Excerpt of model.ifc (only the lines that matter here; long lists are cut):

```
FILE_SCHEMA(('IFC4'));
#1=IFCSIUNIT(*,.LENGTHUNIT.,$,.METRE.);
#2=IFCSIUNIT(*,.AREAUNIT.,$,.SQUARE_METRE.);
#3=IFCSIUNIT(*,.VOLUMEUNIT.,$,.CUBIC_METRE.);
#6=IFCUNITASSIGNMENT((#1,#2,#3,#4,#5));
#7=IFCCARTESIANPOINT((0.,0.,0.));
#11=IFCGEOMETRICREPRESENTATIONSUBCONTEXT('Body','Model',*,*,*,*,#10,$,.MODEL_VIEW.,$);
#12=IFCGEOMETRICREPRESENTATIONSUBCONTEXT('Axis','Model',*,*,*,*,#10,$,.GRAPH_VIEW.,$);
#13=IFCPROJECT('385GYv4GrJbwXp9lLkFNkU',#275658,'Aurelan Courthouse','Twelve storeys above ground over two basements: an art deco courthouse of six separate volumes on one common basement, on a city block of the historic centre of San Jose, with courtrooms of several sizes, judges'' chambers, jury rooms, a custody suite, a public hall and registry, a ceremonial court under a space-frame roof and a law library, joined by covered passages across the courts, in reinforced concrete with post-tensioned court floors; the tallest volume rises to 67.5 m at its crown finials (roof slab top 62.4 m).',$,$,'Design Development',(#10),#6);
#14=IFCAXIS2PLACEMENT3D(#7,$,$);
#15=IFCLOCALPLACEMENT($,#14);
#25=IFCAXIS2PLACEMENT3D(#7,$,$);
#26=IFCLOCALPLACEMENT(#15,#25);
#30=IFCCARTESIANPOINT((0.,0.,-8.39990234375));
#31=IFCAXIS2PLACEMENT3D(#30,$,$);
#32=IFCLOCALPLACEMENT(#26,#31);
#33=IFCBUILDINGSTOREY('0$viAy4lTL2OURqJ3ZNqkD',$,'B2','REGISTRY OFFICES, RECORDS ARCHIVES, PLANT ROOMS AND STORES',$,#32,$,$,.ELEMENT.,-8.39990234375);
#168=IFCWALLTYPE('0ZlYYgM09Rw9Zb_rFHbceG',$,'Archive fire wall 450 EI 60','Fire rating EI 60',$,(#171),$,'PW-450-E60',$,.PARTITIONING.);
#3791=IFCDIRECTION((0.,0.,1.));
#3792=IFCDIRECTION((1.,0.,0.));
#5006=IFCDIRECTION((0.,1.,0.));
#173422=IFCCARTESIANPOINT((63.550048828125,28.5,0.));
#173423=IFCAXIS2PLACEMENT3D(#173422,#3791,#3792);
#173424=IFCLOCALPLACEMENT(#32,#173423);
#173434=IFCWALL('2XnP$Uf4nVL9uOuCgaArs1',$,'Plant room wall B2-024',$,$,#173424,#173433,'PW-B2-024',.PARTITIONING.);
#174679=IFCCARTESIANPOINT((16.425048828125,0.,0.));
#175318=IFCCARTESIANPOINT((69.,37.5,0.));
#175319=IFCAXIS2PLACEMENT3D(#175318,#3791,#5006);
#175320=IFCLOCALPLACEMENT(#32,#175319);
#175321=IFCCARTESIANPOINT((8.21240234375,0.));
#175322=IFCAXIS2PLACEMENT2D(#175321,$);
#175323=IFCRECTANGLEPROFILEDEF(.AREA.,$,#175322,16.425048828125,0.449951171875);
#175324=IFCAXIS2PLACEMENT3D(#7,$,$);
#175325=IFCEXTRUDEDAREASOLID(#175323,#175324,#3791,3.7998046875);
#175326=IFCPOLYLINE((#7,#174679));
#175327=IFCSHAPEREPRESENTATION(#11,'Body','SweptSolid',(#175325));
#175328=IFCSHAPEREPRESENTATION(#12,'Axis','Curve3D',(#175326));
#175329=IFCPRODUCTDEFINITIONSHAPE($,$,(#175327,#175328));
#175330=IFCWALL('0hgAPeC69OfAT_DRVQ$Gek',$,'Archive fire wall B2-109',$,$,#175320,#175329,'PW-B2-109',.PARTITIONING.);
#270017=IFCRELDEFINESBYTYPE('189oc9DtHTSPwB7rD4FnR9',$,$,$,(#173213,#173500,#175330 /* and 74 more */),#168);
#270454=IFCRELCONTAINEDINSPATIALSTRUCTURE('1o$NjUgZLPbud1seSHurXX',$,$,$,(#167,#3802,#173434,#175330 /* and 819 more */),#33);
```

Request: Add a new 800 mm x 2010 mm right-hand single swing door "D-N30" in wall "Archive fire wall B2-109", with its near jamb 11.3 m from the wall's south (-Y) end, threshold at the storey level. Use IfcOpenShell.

```python
import numpy as np
import ifcopenshell
import ifcopenshell.api.feature
import ifcopenshell.api.geometry
import ifcopenshell.api.root
import ifcopenshell.api.spatial
import ifcopenshell.geom
import ifcopenshell.util.element
import ifcopenshell.util.placement
import ifcopenshell.util.representation
import ifcopenshell.util.shape
import ifcopenshell.util.unit

model = ifcopenshell.open("model.ifc")
unit_scale = ifcopenshell.util.unit.calculate_unit_scale(model)
settings = ifcopenshell.geom.settings()


def volume(element):
    """Net volume in cubic metres, openings subtracted."""
    shape = ifcopenshell.geom.create_shape(settings, element)
    return ifcopenshell.util.shape.get_volume(shape.geometry)


wall = model.by_id(175330)
storey = ifcopenshell.util.element.get_container(wall, ifc_class="IfcBuildingStorey")
context = ifcopenshell.util.representation.get_context(model, "Model", "Body", "MODEL_VIEW")
before = volume(wall)

width, height, from_end, sill = 0.8, 2.01, 11.3, 0.0  # metres

# The wall runs along its own X axis, and the end named is its -X end.
wall_shape = ifcopenshell.geom.create_shape(settings, wall)
x, y, z = ifcopenshell.util.shape.get_vertices(wall_shape.geometry).T
start = x.min() + from_end
face, thickness = float(y.min()), float(y.max() - y.min())
wall_matrix = ifcopenshell.util.placement.get_local_placement(wall.ObjectPlacement)
level = ifcopenshell.util.placement.get_local_placement(storey.ObjectPlacement)[2, 3]


def in_wall(x, y):
    """Placement at x, y metres in the wall's axes, at sill height."""
    matrix = wall_matrix.copy()
    matrix[:, 3] = wall_matrix @ np.array([x / unit_scale, y / unit_scale, 0.0, 1.0])
    matrix[2, 3] = level + sill / unit_scale
    return matrix


# Opening: a box that overshoots both wall faces by 50 mm.
opening = ifcopenshell.api.root.create_entity(model, ifc_class="IfcOpeningElement", predefined_type="OPENING")
box = ifcopenshell.api.geometry.add_wall_representation(
    model, context=context, length=width, height=height, thickness=thickness + 0.1
)
ifcopenshell.api.geometry.assign_representation(model, product=opening, representation=box)
ifcopenshell.api.geometry.edit_object_placement(model, product=opening, matrix=in_wall(start, face - 0.05), is_si=False)
ifcopenshell.api.feature.add_feature(model, feature=opening, element=wall)

door = ifcopenshell.api.root.create_entity(model, ifc_class="IfcDoor", name="D-N30", predefined_type="DOOR")
door.OverallWidth, door.OverallHeight = width / unit_scale, height / unit_scale
door.OperationType = "SINGLE_SWING_RIGHT"
body = ifcopenshell.api.geometry.add_door_representation(
    model,
    context=context,
    overall_width=door.OverallWidth,
    overall_height=door.OverallHeight,
    operation_type="SINGLE_SWING_RIGHT",
    lining_properties={"LiningDepth": thickness / unit_scale, "ThresholdDepth": thickness / unit_scale},
)
ifcopenshell.api.geometry.assign_representation(model, product=door, representation=body)
ifcopenshell.api.spatial.assign_container(model, products=[door], relating_structure=storey)
ifcopenshell.api.feature.add_filling(model, opening=opening, element=door)

# The lining spans the wall, so the door starts at the wall face.
ifcopenshell.api.geometry.edit_object_placement(model, product=door, matrix=in_wall(start, face), is_si=False)

after = volume(wall)

print(f"wall volume {before:.3f} -> {after:.3f} m3")

model.write("model_edited.ifc")
```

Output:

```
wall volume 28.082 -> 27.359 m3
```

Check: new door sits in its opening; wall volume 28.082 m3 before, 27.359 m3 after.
